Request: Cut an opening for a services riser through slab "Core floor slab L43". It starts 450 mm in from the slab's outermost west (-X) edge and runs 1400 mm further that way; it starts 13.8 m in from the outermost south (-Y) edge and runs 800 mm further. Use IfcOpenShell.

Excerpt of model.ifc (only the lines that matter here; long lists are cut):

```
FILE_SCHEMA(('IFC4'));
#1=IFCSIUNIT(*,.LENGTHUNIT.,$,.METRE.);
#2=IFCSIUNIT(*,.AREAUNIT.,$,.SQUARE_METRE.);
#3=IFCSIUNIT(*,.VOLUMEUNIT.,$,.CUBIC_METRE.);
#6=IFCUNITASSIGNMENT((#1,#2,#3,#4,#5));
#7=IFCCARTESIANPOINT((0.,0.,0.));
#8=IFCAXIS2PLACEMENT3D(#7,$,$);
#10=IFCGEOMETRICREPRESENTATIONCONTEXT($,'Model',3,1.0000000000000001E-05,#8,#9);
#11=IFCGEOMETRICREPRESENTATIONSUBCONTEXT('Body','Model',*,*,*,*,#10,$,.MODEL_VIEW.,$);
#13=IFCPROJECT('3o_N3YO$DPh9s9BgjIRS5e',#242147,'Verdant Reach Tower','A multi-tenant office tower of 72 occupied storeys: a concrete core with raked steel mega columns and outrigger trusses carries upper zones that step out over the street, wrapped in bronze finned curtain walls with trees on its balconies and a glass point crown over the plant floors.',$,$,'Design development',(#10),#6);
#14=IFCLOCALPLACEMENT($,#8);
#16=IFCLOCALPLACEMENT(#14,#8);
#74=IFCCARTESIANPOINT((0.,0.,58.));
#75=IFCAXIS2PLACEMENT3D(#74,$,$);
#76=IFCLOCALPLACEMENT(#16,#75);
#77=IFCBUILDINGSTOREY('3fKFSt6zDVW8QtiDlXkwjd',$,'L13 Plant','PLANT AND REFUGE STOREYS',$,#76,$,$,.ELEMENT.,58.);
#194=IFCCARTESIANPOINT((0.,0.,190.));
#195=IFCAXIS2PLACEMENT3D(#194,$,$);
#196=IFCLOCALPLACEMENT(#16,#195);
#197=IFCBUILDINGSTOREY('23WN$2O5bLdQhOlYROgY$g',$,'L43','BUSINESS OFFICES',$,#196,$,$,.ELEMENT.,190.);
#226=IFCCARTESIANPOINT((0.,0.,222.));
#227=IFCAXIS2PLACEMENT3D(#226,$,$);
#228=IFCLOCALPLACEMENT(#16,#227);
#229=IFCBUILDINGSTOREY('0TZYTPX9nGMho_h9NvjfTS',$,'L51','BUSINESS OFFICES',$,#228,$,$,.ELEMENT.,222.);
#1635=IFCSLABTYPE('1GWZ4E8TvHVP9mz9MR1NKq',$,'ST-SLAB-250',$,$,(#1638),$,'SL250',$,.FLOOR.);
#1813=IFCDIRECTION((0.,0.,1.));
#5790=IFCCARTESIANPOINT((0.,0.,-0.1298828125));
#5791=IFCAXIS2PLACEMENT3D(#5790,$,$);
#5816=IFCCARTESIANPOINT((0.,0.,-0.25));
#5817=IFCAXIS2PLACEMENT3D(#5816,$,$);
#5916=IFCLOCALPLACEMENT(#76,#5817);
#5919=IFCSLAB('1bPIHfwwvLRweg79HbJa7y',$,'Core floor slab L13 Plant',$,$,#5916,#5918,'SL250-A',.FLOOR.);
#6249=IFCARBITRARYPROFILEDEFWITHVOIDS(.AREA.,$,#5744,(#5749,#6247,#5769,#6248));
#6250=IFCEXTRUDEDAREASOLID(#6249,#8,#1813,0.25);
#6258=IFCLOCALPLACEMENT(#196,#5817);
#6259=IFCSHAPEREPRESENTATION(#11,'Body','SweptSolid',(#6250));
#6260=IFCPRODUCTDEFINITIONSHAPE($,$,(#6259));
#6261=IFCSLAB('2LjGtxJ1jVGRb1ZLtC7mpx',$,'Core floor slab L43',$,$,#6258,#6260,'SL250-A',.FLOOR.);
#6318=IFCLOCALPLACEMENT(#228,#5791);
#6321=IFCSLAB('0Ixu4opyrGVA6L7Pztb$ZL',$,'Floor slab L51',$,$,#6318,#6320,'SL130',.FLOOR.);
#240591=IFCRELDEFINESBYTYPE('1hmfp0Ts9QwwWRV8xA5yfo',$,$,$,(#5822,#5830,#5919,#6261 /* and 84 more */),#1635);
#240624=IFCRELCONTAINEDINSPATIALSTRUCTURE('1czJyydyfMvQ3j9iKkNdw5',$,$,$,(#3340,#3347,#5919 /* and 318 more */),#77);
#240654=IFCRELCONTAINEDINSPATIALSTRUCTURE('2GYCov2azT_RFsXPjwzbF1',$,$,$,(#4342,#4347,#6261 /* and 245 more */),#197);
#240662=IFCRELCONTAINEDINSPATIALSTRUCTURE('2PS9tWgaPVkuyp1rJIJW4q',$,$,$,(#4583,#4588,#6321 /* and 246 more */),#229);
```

```python
import numpy as np
import ifcopenshell
import ifcopenshell.api.feature
import ifcopenshell.api.geometry
import ifcopenshell.api.root
import ifcopenshell.geom
import ifcopenshell.util.placement
import ifcopenshell.util.representation
import ifcopenshell.util.shape
import ifcopenshell.util.unit

model = ifcopenshell.open("model.ifc")
unit_scale = ifcopenshell.util.unit.calculate_unit_scale(model)
settings = ifcopenshell.geom.settings()


def volume(element):
    """Net volume in cubic metres, openings subtracted."""
    shape = ifcopenshell.geom.create_shape(settings, element)
    return ifcopenshell.util.shape.get_volume(shape.geometry)


slab = model.by_guid("2LjGtxJ1jVGRb1ZLtC7mpx")
before = volume(slab)

# Extent in the slab's own axes, in metres. The edges named are its -X and -Y sides.
slab_shape = ifcopenshell.geom.create_shape(settings, slab)
vertices = ifcopenshell.util.shape.get_vertices(slab_shape.geometry)
x_min, y_min, bottom = vertices.min(axis=0)
top = vertices[:, 2].max()

opening = ifcopenshell.api.root.create_entity(model, ifc_class="IfcOpeningElement", name="Services riser opening", predefined_type="OPENING")
context = ifcopenshell.util.representation.get_context(model, "Model", "Body", "MODEL_VIEW")
width, depth = 1.4, 0.8
outline = [(0.0, 0.0), (width, 0.0), (width, depth), (0.0, depth), (0.0, 0.0)]
# Overshoot both faces by 50 mm so the cut is clean.
shape = ifcopenshell.api.geometry.add_slab_representation(
    model, context=context, depth=top - bottom + 0.1, polyline=outline
)
ifcopenshell.api.geometry.assign_representation(model, product=opening, representation=shape)

matrix = ifcopenshell.util.placement.get_local_placement(slab.ObjectPlacement)
matrix[:, 3] = matrix @ np.append(np.array([x_min + 0.45, y_min + 13.8, bottom - 0.05]) / unit_scale, 1.0)
ifcopenshell.api.geometry.edit_object_placement(model, product=opening, matrix=matrix, is_si=False)
ifcopenshell.api.feature.add_feature(model, feature=opening, element=slab)

after = volume(slab)

print(f"slab volume {before:.3f} -> {after:.3f} m3")

model.write("model_edited.ifc")
```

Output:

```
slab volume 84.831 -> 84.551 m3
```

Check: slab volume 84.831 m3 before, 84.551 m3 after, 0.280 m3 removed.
